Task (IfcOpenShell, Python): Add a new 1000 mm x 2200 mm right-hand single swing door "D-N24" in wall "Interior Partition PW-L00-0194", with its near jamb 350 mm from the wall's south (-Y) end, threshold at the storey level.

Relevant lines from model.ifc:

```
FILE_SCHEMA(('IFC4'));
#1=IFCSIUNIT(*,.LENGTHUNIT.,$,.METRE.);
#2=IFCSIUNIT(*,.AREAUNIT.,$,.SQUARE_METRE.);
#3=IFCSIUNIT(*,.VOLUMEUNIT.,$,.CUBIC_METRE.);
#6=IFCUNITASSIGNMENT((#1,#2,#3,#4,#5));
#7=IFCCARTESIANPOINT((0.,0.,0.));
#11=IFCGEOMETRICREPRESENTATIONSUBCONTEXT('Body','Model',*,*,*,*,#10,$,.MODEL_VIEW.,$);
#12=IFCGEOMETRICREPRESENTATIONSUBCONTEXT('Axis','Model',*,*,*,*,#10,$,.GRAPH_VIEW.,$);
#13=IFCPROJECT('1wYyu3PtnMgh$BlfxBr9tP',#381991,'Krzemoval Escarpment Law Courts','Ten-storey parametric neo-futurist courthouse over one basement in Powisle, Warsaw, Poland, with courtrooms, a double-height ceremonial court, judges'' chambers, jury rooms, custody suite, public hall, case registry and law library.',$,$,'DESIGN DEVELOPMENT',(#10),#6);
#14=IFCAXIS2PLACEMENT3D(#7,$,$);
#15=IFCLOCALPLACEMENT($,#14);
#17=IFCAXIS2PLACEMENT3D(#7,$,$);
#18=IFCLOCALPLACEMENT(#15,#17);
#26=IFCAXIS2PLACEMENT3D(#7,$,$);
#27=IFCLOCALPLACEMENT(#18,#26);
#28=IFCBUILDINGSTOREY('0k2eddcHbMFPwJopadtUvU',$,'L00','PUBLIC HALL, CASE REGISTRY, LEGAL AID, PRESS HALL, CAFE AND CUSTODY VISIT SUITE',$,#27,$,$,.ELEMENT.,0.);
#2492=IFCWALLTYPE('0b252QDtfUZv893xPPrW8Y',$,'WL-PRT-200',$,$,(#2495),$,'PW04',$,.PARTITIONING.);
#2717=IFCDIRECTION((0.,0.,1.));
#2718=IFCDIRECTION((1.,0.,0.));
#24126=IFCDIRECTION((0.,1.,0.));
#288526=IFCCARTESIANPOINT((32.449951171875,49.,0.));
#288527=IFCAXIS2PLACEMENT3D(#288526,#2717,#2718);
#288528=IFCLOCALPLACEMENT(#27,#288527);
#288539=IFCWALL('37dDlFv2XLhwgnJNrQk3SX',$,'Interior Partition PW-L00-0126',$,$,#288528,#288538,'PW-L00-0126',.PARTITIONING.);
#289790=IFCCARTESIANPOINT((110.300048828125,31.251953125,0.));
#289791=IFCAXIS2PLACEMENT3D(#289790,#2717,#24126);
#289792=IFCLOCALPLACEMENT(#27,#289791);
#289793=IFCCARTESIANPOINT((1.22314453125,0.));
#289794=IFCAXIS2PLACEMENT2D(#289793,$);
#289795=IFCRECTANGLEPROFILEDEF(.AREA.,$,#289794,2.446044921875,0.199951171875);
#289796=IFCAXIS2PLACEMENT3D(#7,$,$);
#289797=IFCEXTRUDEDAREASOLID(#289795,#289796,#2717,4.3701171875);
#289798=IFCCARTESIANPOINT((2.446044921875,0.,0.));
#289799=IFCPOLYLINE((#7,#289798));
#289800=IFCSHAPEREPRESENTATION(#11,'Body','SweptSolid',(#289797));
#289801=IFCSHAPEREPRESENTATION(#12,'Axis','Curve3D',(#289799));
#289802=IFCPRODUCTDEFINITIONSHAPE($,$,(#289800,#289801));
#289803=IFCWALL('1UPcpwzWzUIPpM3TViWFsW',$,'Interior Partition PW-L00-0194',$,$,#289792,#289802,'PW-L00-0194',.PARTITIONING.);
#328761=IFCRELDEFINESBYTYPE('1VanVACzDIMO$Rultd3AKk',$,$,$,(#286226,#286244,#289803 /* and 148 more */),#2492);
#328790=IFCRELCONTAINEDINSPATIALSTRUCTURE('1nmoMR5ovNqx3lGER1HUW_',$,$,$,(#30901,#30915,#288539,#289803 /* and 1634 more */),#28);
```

```python
import numpy as np
import ifcopenshell
import ifcopenshell.api.feature
import ifcopenshell.api.geometry
import ifcopenshell.api.root
import ifcopenshell.api.spatial
import ifcopenshell.geom
import ifcopenshell.util.element
import ifcopenshell.util.placement
import ifcopenshell.util.representation
import ifcopenshell.util.shape
import ifcopenshell.util.unit

model = ifcopenshell.open("model.ifc")
unit_scale = ifcopenshell.util.unit.calculate_unit_scale(model)
settings = ifcopenshell.geom.settings()


def volume(element):
    """Net volume in cubic metres, openings subtracted."""
    shape = ifcopenshell.geom.create_shape(settings, element)
    return ifcopenshell.util.shape.get_volume(shape.geometry)


wall = model.by_guid("1UPcpwzWzUIPpM3TViWFsW")
storey = ifcopenshell.util.element.get_container(wall, ifc_class="IfcBuildingStorey")
context = ifcopenshell.util.representation.get_context(model, "Model", "Body", "MODEL_VIEW")
before = volume(wall)

width, height, from_end, sill = 1, 2.2, 0.35, 0.0  # metres

# The wall runs along its own X axis, and the end named is its -X end.
wall_shape = ifcopenshell.geom.create_shape(settings, wall)
x, y, z = ifcopenshell.util.shape.get_vertices(wall_shape.geometry).T
start = x.min() + from_end
face, thickness = float(y.min()), float(y.max() - y.min())
wall_matrix = ifcopenshell.util.placement.get_local_placement(wall.ObjectPlacement)
level = ifcopenshell.util.placement.get_local_placement(storey.ObjectPlacement)[2, 3]


def in_wall(x, y):
    """Placement at x, y metres in the wall's axes, at sill height."""
    matrix = wall_matrix.copy()
    matrix[:, 3] = wall_matrix @ np.array([x / unit_scale, y / unit_scale, 0.0, 1.0])
    matrix[2, 3] = level + sill / unit_scale
    return matrix


# Opening: a box that overshoots both wall faces by 50 mm.
opening = ifcopenshell.api.root.create_entity(model, ifc_class="IfcOpeningElement", predefined_type="OPENING")
box = ifcopenshell.api.geometry.add_wall_representation(
    model, context=context, length=width, height=height, thickness=thickness + 0.1
)
ifcopenshell.api.geometry.assign_representation(model, product=opening, representation=box)
ifcopenshell.api.geometry.edit_object_placement(model, product=opening, matrix=in_wall(start, face - 0.05), is_si=False)
ifcopenshell.api.feature.add_feature(model, feature=opening, element=wall)

door = ifcopenshell.api.root.create_entity(model, ifc_class="IfcDoor", name="D-N24", predefined_type="DOOR")
door.OverallWidth, door.OverallHeight = width / unit_scale, height / unit_scale
door.OperationType = "SINGLE_SWING_RIGHT"
body = ifcopenshell.api.geometry.add_door_representation(
    model,
    context=context,
    overall_width=door.OverallWidth,
    overall_height=door.OverallHeight,
    operation_type="SINGLE_SWING_RIGHT",
    lining_properties={"LiningDepth": thickness / unit_scale, "ThresholdDepth": thickness / unit_scale},
)
ifcopenshell.api.geometry.assign_representation(model, product=door, representation=body)
ifcopenshell.api.spatial.assign_container(model, products=[door], relating_structure=storey)
ifcopenshell.api.feature.add_filling(model, opening=opening, element=door)

# The lining spans the wall, so the door starts at the wall face.
ifcopenshell.api.geometry.edit_object_placement(model, product=door, matrix=in_wall(start, face), is_si=False)

after = volume(wall)

print(f"wall volume {before:.3f} -> {after:.3f} m3")

model.write("model_v2.ifc")
```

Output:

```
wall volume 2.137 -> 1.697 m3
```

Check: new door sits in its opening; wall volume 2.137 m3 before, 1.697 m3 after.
